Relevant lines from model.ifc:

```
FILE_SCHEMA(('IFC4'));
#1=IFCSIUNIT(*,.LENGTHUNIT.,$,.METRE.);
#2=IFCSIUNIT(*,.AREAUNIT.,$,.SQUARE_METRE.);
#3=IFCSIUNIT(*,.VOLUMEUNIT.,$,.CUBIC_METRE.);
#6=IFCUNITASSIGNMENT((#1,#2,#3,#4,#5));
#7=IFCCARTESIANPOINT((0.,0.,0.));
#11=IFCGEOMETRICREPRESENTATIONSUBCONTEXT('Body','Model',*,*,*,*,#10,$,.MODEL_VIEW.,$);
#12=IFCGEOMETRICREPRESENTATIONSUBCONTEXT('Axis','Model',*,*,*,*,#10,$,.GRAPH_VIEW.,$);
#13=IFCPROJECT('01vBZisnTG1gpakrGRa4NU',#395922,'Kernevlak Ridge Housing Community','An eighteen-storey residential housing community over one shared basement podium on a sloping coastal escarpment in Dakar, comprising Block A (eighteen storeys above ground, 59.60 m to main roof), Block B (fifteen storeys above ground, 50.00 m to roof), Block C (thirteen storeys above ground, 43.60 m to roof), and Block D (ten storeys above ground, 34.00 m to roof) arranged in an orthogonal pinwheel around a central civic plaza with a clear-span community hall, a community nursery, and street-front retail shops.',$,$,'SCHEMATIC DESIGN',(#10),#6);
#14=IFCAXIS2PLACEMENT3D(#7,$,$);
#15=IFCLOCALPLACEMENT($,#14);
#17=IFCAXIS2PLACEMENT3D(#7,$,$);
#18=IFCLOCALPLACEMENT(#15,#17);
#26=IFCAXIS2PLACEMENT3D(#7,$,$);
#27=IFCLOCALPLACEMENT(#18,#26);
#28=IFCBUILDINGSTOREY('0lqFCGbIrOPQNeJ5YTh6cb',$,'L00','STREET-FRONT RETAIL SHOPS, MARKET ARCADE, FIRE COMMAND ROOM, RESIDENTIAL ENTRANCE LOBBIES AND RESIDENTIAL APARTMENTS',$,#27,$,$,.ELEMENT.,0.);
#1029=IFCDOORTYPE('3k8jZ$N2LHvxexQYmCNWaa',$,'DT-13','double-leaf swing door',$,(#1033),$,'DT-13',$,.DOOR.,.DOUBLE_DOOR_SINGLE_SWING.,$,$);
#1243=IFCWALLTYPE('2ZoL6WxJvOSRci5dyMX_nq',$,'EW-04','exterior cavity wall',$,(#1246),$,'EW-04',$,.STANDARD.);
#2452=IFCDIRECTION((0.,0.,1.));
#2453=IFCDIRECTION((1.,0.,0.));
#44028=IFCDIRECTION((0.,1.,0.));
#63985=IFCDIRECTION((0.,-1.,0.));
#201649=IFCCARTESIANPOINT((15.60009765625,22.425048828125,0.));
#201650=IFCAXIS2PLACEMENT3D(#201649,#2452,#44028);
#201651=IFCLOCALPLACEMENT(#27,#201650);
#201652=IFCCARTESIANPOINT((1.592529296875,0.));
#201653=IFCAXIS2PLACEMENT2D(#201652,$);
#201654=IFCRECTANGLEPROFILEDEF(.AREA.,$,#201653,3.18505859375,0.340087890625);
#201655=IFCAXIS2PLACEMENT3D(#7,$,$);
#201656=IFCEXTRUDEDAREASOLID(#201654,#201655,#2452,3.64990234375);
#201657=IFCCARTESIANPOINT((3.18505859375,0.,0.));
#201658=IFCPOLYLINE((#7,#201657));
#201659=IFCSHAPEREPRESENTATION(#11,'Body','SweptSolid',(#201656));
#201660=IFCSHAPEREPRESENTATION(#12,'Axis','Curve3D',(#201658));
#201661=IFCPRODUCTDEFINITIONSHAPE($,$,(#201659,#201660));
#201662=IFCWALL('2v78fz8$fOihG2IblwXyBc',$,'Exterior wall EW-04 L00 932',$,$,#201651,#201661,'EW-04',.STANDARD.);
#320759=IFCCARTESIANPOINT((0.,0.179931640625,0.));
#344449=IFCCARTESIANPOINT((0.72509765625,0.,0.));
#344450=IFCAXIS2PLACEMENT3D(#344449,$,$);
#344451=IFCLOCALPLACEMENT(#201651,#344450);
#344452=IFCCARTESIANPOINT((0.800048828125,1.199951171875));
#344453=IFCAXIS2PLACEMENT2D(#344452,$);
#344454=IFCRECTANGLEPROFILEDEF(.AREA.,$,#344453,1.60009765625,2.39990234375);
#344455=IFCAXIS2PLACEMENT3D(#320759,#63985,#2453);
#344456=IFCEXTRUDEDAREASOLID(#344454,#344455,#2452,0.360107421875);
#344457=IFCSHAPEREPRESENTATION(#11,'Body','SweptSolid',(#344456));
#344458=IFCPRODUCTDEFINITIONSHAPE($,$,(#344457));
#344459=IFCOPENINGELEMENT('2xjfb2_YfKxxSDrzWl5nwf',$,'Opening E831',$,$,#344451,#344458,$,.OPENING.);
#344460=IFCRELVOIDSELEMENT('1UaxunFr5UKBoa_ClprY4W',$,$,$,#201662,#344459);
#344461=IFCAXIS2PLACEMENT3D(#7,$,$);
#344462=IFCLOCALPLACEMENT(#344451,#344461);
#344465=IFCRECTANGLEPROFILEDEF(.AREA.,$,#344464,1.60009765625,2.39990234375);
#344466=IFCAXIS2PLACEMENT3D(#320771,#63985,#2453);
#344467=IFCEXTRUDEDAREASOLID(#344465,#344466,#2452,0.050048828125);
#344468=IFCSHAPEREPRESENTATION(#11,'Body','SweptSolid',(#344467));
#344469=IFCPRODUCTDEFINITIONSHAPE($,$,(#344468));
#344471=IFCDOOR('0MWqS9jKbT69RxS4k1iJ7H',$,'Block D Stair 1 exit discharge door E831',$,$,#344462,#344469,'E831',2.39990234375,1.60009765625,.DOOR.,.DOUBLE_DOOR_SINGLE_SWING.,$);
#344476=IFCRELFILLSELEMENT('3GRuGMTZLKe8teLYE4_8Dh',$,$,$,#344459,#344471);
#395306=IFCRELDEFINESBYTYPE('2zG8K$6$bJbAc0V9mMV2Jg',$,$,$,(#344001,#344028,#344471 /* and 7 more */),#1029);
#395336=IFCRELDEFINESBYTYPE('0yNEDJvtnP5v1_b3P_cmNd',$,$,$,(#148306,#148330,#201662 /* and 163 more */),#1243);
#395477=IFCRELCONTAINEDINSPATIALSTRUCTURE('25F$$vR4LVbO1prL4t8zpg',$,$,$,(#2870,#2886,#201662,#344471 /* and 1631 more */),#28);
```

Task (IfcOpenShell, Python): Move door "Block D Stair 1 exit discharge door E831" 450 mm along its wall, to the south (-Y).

```python
import ifcopenshell
import ifcopenshell.api.geometry
import ifcopenshell.util.placement

model = ifcopenshell.open("model.ifc")

door = model.by_guid("0MWqS9jKbT69RxS4k1iJ7H")
opening = door.FillsVoids[0].RelatingOpeningElement
wall = opening.VoidsElements[0].RelatingBuildingElement

wall_matrix = ifcopenshell.util.placement.get_local_placement(wall.ObjectPlacement)
shift = wall_matrix[:3, 0] * -0.45
before = ifcopenshell.util.placement.get_local_placement(door.ObjectPlacement)[:3, 3].copy()

# The door is placed relative to its opening, so it follows when the opening moves.
matrix = ifcopenshell.util.placement.get_local_placement(opening.ObjectPlacement)
matrix[:3, 3] += shift
ifcopenshell.api.geometry.edit_object_placement(
    model, product=opening, matrix=matrix, is_si=False, should_transform_children=True
)

after = ifcopenshell.util.placement.get_local_placement(door.ObjectPlacement)[:3, 3]
print("door moved by", (after - before).round(3) + 0.0)

model.write("model-out.ifc")
```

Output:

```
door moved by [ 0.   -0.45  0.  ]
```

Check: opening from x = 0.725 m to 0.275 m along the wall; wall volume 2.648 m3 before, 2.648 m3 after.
